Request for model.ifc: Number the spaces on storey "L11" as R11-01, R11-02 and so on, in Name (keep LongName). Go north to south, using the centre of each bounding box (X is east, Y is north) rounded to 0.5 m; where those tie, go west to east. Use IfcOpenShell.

First a look at what the model holds.

```python
import ifcopenshell
import ifcopenshell.util.element
import ifcopenshell.util.placement

model = ifcopenshell.open("model.ifc")
print(model.schema)
storey = next(s for s in model.by_type("IfcBuildingStorey") if s.Name == "L11")
spaces = [e for e in ifcopenshell.util.element.get_decomposition(storey) if e.is_a("IfcSpace")]
for e in sorted(spaces, key=lambda e: e.id()):
    origin = ifcopenshell.util.placement.get_local_placement(e.ObjectPlacement)[:3, 3]
    print(e.id(), e.Name, e.LongName, origin.round(2) + 0.0, sep=" | ")
```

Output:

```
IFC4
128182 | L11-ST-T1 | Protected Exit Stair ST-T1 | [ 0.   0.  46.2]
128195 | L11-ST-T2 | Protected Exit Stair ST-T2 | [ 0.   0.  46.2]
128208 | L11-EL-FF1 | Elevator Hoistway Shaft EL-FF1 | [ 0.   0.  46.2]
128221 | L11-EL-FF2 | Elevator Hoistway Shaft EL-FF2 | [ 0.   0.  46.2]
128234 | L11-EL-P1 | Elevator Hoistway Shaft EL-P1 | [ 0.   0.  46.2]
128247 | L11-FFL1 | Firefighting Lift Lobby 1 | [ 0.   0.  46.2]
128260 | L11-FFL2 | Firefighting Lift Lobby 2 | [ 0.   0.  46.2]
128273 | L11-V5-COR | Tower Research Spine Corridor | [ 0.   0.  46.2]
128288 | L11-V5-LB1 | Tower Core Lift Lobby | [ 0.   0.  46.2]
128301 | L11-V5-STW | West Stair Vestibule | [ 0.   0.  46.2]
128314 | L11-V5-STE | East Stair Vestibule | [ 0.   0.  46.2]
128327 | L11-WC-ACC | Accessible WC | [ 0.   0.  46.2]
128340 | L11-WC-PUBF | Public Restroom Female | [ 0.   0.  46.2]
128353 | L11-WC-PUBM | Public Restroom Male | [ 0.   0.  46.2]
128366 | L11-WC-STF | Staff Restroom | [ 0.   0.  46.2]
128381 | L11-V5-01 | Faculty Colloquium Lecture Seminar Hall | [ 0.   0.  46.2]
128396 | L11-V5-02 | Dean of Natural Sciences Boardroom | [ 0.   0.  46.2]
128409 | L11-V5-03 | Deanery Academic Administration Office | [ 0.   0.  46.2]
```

```python
import ifcopenshell
import ifcopenshell.geom
import ifcopenshell.util.element
import ifcopenshell.util.shape

model = ifcopenshell.open("model.ifc")
settings = ifcopenshell.geom.settings()
settings.set("use-world-coords", True)


def centre(element):
    shape = ifcopenshell.geom.create_shape(settings, element)
    return ifcopenshell.util.shape.get_bbox_centroid(shape.geometry)


storey = next(s for s in model.by_type("IfcBuildingStorey") if s.Name == "L11")
spaces = [e for e in ifcopenshell.util.element.get_decomposition(storey) if e.is_a("IfcSpace")]

# Insertion points can sit at a corner or the storey origin, so sort by the geometry (in metres).
centres = {e: centre(e) for e in spaces}
spaces.sort(key=lambda e: (-round(centres[e][1] / 0.5), centres[e][0]))

for i, e in enumerate(spaces, start=1):
    number = f"R11-{i:02d}"
    e.Name = number
    print(e.id(), number)

model.write("model_rev.ifc")
```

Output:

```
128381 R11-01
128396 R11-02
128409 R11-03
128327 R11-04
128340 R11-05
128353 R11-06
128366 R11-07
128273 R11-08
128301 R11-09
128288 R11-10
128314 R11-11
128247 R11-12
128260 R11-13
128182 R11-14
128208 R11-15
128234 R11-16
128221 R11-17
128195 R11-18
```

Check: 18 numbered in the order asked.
